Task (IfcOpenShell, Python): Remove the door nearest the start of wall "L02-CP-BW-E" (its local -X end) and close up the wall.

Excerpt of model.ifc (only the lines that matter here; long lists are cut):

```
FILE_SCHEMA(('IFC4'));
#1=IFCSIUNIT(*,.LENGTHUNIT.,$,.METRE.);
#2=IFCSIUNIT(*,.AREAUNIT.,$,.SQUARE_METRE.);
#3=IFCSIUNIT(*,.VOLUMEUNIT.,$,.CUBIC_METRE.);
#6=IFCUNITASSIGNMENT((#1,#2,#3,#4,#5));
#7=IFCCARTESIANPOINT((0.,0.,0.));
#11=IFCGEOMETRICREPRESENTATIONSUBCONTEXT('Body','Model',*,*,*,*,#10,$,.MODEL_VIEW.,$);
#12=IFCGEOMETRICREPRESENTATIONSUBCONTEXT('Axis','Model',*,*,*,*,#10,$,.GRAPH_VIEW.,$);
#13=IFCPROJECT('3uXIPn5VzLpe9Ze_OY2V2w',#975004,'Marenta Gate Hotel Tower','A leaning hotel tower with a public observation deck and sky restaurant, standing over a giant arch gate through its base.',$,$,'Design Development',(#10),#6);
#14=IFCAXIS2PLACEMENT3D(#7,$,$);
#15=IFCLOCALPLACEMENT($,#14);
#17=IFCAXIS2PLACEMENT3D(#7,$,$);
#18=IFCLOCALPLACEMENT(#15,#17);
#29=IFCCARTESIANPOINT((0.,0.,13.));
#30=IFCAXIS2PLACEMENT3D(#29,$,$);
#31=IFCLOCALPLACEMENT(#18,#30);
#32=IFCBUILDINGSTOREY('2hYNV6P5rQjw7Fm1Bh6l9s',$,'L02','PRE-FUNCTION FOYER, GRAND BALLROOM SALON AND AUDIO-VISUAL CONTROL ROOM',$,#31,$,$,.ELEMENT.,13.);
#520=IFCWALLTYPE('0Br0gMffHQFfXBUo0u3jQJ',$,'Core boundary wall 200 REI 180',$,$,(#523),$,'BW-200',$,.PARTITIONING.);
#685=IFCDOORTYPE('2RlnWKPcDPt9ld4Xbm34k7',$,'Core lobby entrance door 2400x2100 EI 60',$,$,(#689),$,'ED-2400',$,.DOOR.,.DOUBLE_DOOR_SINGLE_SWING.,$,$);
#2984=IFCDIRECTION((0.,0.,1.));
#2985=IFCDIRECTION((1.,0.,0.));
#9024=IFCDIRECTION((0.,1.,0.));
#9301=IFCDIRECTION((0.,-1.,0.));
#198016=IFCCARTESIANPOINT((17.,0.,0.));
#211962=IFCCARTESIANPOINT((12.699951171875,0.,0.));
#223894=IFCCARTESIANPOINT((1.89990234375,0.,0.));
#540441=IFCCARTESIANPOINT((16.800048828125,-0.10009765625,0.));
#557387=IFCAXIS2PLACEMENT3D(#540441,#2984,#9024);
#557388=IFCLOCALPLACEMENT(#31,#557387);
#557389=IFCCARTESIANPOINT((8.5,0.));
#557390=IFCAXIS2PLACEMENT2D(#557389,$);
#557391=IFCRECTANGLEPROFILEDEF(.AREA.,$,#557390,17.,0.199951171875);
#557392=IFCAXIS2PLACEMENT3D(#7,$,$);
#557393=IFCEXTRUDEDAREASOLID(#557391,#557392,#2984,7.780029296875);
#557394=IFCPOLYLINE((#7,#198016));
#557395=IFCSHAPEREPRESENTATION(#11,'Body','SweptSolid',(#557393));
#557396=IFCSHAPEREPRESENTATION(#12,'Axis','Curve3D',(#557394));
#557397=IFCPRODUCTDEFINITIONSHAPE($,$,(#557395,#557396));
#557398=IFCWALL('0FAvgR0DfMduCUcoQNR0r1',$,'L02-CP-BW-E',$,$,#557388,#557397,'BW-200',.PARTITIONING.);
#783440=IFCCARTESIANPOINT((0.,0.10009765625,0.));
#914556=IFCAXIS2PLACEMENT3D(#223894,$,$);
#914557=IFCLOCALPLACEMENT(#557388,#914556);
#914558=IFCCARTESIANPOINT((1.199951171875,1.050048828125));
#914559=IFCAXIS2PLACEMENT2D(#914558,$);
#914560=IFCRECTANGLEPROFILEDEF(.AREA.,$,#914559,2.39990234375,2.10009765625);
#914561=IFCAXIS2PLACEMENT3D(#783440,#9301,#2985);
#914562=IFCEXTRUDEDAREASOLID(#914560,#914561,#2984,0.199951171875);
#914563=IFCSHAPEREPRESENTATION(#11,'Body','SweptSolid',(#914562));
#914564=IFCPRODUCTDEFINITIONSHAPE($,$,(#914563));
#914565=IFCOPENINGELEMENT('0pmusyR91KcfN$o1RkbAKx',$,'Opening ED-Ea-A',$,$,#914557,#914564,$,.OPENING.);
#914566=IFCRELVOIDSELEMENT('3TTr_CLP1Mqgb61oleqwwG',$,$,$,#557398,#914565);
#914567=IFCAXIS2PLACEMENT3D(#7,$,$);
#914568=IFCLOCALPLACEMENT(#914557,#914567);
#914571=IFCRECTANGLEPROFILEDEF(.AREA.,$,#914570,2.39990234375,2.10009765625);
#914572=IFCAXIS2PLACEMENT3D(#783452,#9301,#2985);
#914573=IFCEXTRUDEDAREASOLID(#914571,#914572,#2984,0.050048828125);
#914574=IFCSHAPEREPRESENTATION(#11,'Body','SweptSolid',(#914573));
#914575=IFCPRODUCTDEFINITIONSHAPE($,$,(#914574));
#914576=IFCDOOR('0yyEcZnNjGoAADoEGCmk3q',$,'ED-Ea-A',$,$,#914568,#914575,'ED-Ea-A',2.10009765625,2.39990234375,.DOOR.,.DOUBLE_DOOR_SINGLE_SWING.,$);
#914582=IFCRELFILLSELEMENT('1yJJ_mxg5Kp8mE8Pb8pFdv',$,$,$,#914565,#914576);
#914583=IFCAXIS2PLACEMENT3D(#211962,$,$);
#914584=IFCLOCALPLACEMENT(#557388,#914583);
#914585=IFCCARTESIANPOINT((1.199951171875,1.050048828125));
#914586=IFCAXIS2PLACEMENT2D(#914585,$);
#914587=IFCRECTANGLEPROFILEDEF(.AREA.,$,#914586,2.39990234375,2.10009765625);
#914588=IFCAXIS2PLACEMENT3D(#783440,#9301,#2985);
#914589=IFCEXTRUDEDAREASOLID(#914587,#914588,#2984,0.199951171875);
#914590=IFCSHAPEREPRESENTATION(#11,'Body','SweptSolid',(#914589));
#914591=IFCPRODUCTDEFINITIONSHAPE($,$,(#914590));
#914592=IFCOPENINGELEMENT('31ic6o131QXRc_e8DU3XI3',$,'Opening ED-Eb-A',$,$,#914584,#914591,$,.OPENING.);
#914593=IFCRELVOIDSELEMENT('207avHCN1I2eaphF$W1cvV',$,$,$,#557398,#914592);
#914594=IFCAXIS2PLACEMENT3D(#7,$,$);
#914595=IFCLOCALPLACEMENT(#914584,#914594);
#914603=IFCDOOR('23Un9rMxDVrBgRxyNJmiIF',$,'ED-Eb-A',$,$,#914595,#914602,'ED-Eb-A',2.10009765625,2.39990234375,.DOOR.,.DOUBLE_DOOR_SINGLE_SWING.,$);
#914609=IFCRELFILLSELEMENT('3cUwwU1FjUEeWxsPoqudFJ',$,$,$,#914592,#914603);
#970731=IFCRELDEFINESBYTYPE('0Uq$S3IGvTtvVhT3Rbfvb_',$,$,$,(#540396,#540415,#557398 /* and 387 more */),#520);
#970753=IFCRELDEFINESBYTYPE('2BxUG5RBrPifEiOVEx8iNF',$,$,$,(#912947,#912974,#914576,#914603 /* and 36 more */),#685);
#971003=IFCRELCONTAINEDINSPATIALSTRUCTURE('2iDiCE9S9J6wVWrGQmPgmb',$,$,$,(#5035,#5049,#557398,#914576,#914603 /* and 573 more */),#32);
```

```python
import ifcopenshell
import ifcopenshell.api.feature
import ifcopenshell.api.root
import ifcopenshell.geom
import ifcopenshell.util.shape

model = ifcopenshell.open("model.ifc")
settings = ifcopenshell.geom.settings()


def volume(element):
    """Net volume in cubic metres, openings subtracted."""
    shape = ifcopenshell.geom.create_shape(settings, element)
    return ifcopenshell.util.shape.get_volume(shape.geometry)


door = model.by_guid("0yyEcZnNjGoAADoEGCmk3q")
opening = door.FillsVoids[0].RelatingOpeningElement
wall = opening.VoidsElements[0].RelatingBuildingElement
before = volume(wall)

ifcopenshell.api.root.remove_product(model, product=door)
ifcopenshell.api.feature.remove_feature(model, feature=opening)

after = volume(wall)

print(f"wall volume {before:.3f} -> {after:.3f} m3")

model.write("model_v2.ifc")
```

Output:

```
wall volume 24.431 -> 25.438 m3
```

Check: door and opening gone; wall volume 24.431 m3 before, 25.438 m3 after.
